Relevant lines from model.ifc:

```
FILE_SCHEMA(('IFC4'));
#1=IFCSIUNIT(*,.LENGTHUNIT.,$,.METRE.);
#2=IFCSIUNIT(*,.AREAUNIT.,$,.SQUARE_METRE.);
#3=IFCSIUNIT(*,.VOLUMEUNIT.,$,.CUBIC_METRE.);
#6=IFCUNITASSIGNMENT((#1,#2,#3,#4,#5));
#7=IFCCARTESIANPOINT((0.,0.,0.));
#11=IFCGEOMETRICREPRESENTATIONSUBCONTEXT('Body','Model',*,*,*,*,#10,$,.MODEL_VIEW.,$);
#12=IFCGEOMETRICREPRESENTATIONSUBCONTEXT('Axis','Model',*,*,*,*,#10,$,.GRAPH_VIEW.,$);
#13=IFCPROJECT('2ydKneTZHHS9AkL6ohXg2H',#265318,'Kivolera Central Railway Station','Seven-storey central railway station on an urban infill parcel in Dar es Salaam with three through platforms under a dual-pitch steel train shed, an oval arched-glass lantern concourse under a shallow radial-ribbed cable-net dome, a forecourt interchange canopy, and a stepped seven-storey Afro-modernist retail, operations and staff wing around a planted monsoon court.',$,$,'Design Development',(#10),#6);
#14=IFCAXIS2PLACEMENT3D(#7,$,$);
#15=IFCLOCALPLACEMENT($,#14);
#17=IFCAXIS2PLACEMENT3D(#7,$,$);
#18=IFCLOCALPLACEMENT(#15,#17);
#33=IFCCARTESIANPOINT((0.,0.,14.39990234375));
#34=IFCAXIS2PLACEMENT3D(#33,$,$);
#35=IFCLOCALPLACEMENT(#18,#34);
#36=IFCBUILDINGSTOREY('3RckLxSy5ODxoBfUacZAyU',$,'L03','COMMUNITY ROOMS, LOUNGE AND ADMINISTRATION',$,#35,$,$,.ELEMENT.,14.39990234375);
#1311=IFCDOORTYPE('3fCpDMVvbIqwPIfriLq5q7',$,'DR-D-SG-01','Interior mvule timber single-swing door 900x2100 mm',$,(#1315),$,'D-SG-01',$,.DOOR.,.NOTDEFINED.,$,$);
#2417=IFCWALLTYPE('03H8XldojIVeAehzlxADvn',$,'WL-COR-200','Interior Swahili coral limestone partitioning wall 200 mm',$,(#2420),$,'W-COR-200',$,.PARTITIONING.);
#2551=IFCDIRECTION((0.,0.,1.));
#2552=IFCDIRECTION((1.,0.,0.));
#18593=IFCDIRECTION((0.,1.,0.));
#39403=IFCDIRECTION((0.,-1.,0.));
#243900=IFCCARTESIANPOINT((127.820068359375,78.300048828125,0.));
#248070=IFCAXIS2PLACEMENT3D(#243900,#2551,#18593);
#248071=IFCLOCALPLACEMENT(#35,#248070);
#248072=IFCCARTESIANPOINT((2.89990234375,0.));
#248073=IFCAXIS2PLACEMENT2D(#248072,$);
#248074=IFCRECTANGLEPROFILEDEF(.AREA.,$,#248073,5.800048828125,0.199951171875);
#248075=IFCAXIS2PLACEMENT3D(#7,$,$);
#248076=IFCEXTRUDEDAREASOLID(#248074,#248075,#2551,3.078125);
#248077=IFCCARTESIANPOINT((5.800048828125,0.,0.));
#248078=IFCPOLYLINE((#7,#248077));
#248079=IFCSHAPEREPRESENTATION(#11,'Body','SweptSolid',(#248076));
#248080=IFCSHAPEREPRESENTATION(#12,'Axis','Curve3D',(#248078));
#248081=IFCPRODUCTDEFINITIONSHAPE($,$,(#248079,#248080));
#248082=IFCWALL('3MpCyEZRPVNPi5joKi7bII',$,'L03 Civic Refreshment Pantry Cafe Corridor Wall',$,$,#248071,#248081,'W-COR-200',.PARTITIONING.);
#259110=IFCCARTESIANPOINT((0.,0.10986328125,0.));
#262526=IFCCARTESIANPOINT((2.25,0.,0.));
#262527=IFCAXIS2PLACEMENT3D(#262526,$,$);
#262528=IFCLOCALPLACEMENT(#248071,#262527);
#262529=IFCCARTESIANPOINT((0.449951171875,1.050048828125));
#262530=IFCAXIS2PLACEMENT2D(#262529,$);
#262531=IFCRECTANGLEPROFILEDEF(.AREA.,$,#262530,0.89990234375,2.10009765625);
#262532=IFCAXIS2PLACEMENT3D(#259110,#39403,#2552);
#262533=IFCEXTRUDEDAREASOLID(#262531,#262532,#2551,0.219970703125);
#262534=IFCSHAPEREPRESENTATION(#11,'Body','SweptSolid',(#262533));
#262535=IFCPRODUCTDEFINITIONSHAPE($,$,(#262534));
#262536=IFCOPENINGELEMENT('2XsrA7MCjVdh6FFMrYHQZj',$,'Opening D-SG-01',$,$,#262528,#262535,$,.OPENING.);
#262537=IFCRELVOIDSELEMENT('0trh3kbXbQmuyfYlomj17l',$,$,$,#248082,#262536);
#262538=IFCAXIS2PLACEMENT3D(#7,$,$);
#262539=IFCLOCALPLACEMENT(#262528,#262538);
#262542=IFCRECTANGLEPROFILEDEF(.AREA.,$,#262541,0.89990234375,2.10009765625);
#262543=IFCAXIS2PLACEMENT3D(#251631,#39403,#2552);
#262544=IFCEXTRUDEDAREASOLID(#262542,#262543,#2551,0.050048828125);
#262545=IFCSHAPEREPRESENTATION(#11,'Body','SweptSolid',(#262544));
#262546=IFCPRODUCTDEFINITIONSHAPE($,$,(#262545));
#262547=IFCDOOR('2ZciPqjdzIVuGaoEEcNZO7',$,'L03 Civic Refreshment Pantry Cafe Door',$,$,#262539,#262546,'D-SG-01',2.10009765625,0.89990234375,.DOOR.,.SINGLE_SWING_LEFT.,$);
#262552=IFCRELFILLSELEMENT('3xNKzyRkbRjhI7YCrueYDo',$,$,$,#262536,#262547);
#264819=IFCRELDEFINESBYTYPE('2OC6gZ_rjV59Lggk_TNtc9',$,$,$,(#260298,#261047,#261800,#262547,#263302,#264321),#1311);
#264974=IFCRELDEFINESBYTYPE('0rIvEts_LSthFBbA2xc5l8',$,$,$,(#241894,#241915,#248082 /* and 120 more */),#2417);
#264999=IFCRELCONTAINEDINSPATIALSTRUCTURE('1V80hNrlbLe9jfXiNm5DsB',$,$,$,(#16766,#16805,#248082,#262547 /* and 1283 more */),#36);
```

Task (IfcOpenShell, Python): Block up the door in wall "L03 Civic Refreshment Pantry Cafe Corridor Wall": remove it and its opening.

```python
import ifcopenshell
import ifcopenshell.api.feature
import ifcopenshell.api.root
import ifcopenshell.geom
import ifcopenshell.util.shape

model = ifcopenshell.open("model.ifc")
settings = ifcopenshell.geom.settings()


def volume(element):
    """Net volume in cubic metres, openings subtracted."""
    shape = ifcopenshell.geom.create_shape(settings, element)
    return ifcopenshell.util.shape.get_volume(shape.geometry)


door = model.by_guid("2ZciPqjdzIVuGaoEEcNZO7")
opening = door.FillsVoids[0].RelatingOpeningElement
wall = opening.VoidsElements[0].RelatingBuildingElement
before = volume(wall)

ifcopenshell.api.root.remove_product(model, product=door)
ifcopenshell.api.feature.remove_feature(model, feature=opening)

after = volume(wall)

print(f"wall volume {before:.3f} -> {after:.3f} m3")

model.write("model-out.ifc")
```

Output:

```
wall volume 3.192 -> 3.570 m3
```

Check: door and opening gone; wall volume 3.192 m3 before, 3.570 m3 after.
